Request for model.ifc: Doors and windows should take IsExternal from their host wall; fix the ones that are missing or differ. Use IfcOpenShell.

First a look at what the model holds.

```python
import ifcopenshell
import ifcopenshell.util.element

model = ifcopenshell.open("model.ifc")
print(model.schema)
seen = {}
for e in model.by_type("IfcDoor") + model.by_type("IfcWindow"):
    if not e.FillsVoids:
        continue
    host = e.FillsVoids[0].RelatingOpeningElement.VoidsElements[0].RelatingBuildingElement
    own = ifcopenshell.util.element.get_pset(e, f"Pset_{e.is_a()[3:].removesuffix('StandardCase')}Common", "IsExternal")
    wall = ifcopenshell.util.element.get_pset(host, "Pset_WallCommon", "IsExternal")
    seen[e.is_a(), own, wall] = seen.get((e.is_a(), own, wall), 0) + 1
for (cls, own, wall), count in sorted(seen.items(), key=str):
    print(count, cls, "IsExternal:", own, "| host wall:", wall)
```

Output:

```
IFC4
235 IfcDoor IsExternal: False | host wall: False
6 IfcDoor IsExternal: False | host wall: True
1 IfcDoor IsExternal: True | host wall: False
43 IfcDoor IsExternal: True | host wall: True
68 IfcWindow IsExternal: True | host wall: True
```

```python
import ifcopenshell
import ifcopenshell.api.pset
import ifcopenshell.util.element

model = ifcopenshell.open("model.ifc")

count = 0
for ifc_class, pset_name in (("IfcDoor", "Pset_DoorCommon"), ("IfcWindow", "Pset_WindowCommon")):
    for e in model.by_type(ifc_class):
        if not e.FillsVoids:
            continue
        host = e.FillsVoids[0].RelatingOpeningElement.VoidsElements[0].RelatingBuildingElement
        external = ifcopenshell.util.element.get_pset(host, "Pset_WallCommon", "IsExternal")
        if external is None or ifcopenshell.util.element.get_pset(e, pset_name, "IsExternal") == external:
            continue
        pset = ifcopenshell.api.pset.add_pset(model, product=e, name=pset_name)
        ifcopenshell.api.pset.edit_pset(model, pset=pset, properties={"IsExternal": external})
        count += 1

print(count, "updated")

model.write("model_rev.ifc")
```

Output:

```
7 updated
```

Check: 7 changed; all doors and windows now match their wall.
